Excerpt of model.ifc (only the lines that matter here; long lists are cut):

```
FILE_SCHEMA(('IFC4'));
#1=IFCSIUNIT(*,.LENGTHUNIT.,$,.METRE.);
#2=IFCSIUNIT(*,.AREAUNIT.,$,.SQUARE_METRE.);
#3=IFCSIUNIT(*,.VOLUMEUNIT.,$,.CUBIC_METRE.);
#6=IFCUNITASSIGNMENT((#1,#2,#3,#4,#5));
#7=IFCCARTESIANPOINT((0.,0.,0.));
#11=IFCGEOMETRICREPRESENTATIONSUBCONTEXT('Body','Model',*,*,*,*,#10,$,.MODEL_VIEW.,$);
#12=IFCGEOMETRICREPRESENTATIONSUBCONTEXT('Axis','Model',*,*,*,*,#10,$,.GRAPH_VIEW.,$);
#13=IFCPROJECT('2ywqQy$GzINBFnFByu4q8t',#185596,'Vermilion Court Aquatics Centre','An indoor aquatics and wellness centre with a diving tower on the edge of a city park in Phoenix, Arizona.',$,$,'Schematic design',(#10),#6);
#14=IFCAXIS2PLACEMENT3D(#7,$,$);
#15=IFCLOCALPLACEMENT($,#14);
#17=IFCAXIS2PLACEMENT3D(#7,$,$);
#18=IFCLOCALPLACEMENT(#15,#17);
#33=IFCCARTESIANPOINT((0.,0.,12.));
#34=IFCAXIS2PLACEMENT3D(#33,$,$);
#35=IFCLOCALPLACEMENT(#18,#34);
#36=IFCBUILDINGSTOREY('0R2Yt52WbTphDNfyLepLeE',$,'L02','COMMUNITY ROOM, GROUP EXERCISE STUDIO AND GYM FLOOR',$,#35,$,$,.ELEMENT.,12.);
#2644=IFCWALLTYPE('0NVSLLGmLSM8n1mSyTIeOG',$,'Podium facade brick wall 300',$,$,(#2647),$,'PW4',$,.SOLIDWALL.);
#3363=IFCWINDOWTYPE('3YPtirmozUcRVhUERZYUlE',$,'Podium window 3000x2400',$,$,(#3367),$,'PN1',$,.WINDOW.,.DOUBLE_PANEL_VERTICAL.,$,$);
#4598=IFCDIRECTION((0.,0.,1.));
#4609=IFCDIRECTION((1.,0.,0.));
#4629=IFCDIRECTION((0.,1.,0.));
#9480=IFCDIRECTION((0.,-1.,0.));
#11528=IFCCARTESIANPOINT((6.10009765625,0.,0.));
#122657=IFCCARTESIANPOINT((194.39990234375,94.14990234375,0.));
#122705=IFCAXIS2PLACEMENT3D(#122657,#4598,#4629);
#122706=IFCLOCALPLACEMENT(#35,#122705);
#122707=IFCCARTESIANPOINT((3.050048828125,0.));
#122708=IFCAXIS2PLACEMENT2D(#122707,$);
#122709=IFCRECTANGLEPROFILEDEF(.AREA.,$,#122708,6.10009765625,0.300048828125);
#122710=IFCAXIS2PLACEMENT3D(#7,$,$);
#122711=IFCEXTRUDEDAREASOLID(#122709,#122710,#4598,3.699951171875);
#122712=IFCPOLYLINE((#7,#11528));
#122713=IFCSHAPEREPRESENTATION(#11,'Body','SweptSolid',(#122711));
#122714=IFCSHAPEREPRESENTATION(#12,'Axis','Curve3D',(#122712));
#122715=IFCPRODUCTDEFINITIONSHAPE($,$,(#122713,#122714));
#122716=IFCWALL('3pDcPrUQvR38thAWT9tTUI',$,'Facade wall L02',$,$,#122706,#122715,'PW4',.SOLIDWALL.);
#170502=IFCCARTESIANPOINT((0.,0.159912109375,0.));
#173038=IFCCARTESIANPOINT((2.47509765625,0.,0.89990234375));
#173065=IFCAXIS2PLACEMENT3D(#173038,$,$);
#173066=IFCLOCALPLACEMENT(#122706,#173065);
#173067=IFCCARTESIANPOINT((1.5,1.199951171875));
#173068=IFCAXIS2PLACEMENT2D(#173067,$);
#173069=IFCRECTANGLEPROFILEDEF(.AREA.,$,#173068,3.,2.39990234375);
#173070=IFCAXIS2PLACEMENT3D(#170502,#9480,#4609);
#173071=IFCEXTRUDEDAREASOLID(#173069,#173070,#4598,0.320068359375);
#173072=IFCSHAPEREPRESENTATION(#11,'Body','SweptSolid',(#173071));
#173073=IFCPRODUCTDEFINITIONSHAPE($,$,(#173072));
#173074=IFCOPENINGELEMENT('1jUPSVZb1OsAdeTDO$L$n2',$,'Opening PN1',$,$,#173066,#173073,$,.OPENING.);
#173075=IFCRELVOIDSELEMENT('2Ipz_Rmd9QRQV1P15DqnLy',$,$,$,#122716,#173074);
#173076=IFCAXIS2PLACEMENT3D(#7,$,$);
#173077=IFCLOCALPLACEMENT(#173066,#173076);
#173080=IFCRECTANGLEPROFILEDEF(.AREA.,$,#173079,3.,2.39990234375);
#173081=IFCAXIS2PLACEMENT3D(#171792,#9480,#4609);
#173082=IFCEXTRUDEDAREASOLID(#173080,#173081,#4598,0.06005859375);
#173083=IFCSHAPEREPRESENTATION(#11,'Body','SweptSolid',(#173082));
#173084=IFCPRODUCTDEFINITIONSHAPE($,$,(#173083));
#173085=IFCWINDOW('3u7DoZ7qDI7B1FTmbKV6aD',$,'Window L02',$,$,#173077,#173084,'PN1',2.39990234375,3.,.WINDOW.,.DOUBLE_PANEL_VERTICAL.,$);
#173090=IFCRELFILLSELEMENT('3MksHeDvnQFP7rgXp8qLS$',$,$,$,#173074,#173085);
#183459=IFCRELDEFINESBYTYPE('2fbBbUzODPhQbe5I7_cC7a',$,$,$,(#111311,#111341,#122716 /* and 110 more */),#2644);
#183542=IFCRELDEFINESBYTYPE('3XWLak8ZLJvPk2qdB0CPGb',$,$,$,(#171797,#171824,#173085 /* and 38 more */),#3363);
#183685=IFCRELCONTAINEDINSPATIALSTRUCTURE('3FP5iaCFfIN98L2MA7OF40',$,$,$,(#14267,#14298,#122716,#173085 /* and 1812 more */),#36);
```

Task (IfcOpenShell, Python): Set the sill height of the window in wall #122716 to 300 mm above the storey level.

```python
import numpy as np
import ifcopenshell
import ifcopenshell.api.geometry
import ifcopenshell.geom
import ifcopenshell.util.element
import ifcopenshell.util.placement
import ifcopenshell.util.shape
import ifcopenshell.util.unit

model = ifcopenshell.open("model.ifc")
unit_scale = ifcopenshell.util.unit.calculate_unit_scale(model)

window = model.by_id(173085)
opening = window.FillsVoids[0].RelatingOpeningElement
storey = ifcopenshell.util.element.get_container(window, ifc_class="IfcBuildingStorey")
level = ifcopenshell.util.placement.get_local_placement(storey.ObjectPlacement)[2, 3]

# The opening's origin need not be at the sill, so measure its lowest point.
shape = ifcopenshell.geom.create_shape(ifcopenshell.geom.settings(), opening)
bottom = ifcopenshell.util.shape.get_shape_bottom_elevation(shape, shape.geometry) / unit_scale
dz = level + 0.3 - bottom

shift = np.array([0.0, 0.0, dz])
# The window is placed relative to its opening, so it follows when the opening moves.
matrix = ifcopenshell.util.placement.get_local_placement(opening.ObjectPlacement)
matrix[:3, 3] += shift
ifcopenshell.api.geometry.edit_object_placement(
    model, product=opening, matrix=matrix, is_si=False, should_transform_children=True
)

print(f"moved by {dz * unit_scale:+.3f} m")

model.write("model_updated.ifc")
```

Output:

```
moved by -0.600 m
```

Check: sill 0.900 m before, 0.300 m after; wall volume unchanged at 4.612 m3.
